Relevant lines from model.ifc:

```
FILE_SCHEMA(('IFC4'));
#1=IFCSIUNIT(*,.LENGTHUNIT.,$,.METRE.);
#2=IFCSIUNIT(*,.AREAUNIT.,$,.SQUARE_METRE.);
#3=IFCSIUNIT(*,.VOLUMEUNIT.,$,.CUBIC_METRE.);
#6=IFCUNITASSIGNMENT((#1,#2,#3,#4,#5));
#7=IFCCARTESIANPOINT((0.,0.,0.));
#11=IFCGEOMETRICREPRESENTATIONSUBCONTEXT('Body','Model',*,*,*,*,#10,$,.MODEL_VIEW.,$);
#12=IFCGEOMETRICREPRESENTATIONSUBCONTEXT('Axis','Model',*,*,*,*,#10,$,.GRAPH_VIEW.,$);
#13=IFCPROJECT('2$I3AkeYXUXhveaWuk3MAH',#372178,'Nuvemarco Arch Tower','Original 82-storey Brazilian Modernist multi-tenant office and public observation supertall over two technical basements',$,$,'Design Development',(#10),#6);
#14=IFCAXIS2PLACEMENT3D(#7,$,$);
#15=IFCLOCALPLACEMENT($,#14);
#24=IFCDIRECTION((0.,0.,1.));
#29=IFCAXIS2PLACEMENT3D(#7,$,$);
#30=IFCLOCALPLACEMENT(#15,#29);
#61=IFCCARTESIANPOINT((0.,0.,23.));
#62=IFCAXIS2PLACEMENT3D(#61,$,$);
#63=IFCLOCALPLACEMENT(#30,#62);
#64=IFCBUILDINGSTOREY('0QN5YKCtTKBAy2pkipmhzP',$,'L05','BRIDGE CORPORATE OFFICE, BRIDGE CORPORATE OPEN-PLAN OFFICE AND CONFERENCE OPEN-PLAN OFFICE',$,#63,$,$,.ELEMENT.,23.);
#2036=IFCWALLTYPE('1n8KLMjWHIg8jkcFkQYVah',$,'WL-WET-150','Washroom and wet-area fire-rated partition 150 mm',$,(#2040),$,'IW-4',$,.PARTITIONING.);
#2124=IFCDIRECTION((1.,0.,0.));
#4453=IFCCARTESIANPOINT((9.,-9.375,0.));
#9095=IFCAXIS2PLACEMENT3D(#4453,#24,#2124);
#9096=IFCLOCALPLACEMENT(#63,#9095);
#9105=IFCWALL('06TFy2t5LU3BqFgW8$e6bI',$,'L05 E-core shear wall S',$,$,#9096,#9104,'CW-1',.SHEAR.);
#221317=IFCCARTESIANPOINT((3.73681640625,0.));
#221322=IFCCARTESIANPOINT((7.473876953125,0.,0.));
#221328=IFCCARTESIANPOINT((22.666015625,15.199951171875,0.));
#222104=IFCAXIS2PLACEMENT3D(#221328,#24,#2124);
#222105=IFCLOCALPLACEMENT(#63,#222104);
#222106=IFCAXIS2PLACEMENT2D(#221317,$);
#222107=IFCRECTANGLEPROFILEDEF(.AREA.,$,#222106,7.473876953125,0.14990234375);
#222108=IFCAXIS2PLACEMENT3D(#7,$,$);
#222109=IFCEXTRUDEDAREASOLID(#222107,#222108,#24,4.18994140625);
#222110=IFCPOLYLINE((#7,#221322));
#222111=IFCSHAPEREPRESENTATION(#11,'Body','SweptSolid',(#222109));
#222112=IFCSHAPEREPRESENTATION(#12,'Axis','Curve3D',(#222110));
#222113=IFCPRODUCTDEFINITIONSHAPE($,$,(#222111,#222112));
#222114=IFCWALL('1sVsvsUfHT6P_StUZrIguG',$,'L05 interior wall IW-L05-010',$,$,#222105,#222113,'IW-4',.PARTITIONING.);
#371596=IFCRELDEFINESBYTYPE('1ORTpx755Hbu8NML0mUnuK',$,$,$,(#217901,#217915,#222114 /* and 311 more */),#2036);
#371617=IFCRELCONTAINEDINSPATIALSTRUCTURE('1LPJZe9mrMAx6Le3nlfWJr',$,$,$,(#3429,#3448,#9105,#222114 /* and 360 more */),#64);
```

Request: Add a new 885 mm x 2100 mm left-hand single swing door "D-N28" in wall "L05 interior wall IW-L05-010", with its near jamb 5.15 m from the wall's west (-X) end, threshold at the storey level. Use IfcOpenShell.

```python
import numpy as np
import ifcopenshell
import ifcopenshell.api.feature
import ifcopenshell.api.geometry
import ifcopenshell.api.root
import ifcopenshell.api.spatial
import ifcopenshell.geom
import ifcopenshell.util.element
import ifcopenshell.util.placement
import ifcopenshell.util.representation
import ifcopenshell.util.shape
import ifcopenshell.util.unit

model = ifcopenshell.open("model.ifc")
unit_scale = ifcopenshell.util.unit.calculate_unit_scale(model)
settings = ifcopenshell.geom.settings()


def volume(element):
    """Net volume in cubic metres, openings subtracted."""
    shape = ifcopenshell.geom.create_shape(settings, element)
    return ifcopenshell.util.shape.get_volume(shape.geometry)


wall = model.by_guid("1sVsvsUfHT6P_StUZrIguG")
storey = ifcopenshell.util.element.get_container(wall, ifc_class="IfcBuildingStorey")
context = ifcopenshell.util.representation.get_context(model, "Model", "Body", "MODEL_VIEW")
before = volume(wall)

width, height, from_end, sill = 0.885, 2.1, 5.15, 0.0  # metres

# The wall runs along its own X axis, and the end named is its -X end.
wall_shape = ifcopenshell.geom.create_shape(settings, wall)
x, y, z = ifcopenshell.util.shape.get_vertices(wall_shape.geometry).T
start = x.min() + from_end
face, thickness = float(y.min()), float(y.max() - y.min())
wall_matrix = ifcopenshell.util.placement.get_local_placement(wall.ObjectPlacement)
level = ifcopenshell.util.placement.get_local_placement(storey.ObjectPlacement)[2, 3]


def in_wall(x, y):
    """Placement at x, y metres in the wall's axes, at sill height."""
    matrix = wall_matrix.copy()
    matrix[:, 3] = wall_matrix @ np.array([x / unit_scale, y / unit_scale, 0.0, 1.0])
    matrix[2, 3] = level + sill / unit_scale
    return matrix


# Opening: a box that overshoots both wall faces by 50 mm.
opening = ifcopenshell.api.root.create_entity(model, ifc_class="IfcOpeningElement", predefined_type="OPENING")
box = ifcopenshell.api.geometry.add_wall_representation(
    model, context=context, length=width, height=height, thickness=thickness + 0.1
)
ifcopenshell.api.geometry.assign_representation(model, product=opening, representation=box)
ifcopenshell.api.geometry.edit_object_placement(model, product=opening, matrix=in_wall(start, face - 0.05), is_si=False)
ifcopenshell.api.feature.add_feature(model, feature=opening, element=wall)

door = ifcopenshell.api.root.create_entity(model, ifc_class="IfcDoor", name="D-N28", predefined_type="DOOR")
door.OverallWidth, door.OverallHeight = width / unit_scale, height / unit_scale
door.OperationType = "SINGLE_SWING_LEFT"
body = ifcopenshell.api.geometry.add_door_representation(
    model,
    context=context,
    overall_width=door.OverallWidth,
    overall_height=door.OverallHeight,
    operation_type="SINGLE_SWING_LEFT",
    lining_properties={"LiningDepth": thickness / unit_scale, "ThresholdDepth": thickness / unit_scale},
)
ifcopenshell.api.geometry.assign_representation(model, product=door, representation=body)
ifcopenshell.api.spatial.assign_container(model, products=[door], relating_structure=storey)
ifcopenshell.api.feature.add_filling(model, opening=opening, element=door)

# The lining spans the wall, so the door starts at the wall face.
ifcopenshell.api.geometry.edit_object_placement(model, product=door, matrix=in_wall(start, face), is_si=False)

after = volume(wall)

print(f"wall volume {before:.3f} -> {after:.3f} m3")

model.write("model_edited.ifc")
```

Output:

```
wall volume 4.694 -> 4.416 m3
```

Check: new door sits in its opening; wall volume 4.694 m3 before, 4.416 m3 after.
